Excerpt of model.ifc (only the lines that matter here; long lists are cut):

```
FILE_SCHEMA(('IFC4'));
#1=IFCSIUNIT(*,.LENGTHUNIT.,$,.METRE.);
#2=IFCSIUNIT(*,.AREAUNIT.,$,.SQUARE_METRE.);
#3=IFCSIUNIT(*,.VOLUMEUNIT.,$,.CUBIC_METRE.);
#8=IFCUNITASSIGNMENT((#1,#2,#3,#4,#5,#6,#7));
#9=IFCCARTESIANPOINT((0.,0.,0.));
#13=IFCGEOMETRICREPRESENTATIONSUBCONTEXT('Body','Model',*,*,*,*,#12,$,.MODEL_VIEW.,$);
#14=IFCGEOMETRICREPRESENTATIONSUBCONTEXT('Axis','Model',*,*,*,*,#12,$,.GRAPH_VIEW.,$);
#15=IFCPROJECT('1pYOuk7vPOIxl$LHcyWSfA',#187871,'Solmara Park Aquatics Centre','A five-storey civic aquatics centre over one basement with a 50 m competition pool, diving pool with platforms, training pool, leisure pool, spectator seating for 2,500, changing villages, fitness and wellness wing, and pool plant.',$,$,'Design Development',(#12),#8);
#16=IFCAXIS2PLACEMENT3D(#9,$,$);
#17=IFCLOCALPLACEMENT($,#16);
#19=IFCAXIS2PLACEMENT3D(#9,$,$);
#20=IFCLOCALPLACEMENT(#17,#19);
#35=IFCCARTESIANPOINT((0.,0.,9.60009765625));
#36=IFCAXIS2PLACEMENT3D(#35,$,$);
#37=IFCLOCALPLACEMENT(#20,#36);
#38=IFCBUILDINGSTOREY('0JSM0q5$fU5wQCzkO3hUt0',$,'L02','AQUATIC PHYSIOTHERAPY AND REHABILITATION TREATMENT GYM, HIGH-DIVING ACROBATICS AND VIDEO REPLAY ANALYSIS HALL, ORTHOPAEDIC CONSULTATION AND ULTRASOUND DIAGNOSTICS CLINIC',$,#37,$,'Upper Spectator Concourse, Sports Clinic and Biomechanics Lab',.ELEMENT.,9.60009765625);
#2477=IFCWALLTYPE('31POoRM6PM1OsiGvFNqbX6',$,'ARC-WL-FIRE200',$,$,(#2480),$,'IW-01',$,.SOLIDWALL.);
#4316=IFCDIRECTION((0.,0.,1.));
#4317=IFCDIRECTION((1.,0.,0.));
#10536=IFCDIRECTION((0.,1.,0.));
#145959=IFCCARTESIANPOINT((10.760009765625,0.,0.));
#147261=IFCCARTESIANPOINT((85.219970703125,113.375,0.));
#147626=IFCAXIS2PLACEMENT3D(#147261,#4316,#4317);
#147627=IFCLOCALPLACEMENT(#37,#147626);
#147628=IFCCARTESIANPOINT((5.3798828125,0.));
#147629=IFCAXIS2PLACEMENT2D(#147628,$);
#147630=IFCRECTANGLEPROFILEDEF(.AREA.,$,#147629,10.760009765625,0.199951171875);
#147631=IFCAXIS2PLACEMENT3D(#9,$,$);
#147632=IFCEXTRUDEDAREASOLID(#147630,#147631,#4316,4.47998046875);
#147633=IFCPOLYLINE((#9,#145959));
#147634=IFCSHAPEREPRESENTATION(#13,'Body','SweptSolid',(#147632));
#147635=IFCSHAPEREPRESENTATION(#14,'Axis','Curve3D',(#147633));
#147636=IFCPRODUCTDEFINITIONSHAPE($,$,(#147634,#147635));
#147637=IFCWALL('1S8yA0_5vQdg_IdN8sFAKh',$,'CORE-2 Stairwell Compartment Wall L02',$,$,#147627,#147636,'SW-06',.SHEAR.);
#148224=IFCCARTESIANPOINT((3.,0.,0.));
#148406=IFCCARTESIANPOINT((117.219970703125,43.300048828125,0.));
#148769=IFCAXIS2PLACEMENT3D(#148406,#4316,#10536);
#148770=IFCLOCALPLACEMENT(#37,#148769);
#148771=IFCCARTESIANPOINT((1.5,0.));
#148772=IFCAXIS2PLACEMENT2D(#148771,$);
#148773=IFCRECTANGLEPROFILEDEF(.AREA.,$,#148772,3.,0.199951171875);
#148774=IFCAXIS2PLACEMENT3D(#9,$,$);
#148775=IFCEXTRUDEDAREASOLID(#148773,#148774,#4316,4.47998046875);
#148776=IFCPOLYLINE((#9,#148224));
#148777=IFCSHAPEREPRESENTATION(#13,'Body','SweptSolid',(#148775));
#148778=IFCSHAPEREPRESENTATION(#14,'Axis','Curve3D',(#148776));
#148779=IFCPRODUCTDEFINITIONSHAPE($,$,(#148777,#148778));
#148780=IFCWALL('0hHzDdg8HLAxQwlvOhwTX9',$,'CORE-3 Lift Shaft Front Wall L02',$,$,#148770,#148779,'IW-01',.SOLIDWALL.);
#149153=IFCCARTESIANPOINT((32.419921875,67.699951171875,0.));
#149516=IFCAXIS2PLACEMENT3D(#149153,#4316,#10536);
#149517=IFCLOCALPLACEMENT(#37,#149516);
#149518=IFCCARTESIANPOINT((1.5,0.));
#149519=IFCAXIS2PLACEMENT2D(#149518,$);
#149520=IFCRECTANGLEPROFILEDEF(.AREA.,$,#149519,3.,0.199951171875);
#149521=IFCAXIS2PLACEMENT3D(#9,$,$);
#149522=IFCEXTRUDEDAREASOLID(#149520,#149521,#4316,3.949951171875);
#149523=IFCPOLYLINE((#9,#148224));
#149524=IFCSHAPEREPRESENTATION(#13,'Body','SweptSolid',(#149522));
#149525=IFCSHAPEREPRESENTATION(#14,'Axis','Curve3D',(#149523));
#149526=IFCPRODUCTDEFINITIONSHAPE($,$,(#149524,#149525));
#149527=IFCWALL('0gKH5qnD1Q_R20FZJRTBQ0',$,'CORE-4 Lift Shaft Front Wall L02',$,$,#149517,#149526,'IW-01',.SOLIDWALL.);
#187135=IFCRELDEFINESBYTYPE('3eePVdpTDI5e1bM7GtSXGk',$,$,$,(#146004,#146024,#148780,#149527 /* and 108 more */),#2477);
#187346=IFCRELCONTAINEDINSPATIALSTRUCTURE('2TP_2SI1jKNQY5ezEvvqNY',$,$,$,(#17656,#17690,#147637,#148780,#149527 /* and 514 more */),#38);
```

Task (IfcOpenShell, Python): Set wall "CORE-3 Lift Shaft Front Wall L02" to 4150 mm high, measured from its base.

```python
import ifcopenshell
import ifcopenshell.geom
import ifcopenshell.util.representation
import ifcopenshell.util.shape
import ifcopenshell.util.unit

model = ifcopenshell.open("model.ifc")
unit_scale = ifcopenshell.util.unit.calculate_unit_scale(model)
settings = ifcopenshell.geom.settings()


def volume(element):
    """Net volume in cubic metres, openings subtracted."""
    shape = ifcopenshell.geom.create_shape(settings, element)
    return ifcopenshell.util.shape.get_volume(shape.geometry)


wall = model.by_id(148780)
before = volume(wall)

body = ifcopenshell.util.representation.get_representation(wall, "Model", "Body")
solid = body.Items[0]
old_height = solid.Depth
solid.Depth = 4.15 / unit_scale
after = volume(wall)

print(f"height {old_height:g} -> {solid.Depth:g}, volume {before:.3f} -> {after:.3f} m3")

model.write("model_edited.ifc")
```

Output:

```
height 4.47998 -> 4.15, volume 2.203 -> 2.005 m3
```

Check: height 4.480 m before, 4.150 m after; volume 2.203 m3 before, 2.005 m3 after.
